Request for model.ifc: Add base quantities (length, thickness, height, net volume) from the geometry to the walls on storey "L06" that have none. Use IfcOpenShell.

First a look at what the model holds.

```python
import ifcopenshell
import ifcopenshell.util.element
import ifcopenshell.util.unit

model = ifcopenshell.open("model.ifc")
print(model.schema)
for unit_type in ("LENGTHUNIT", "AREAUNIT", "VOLUMEUNIT"):
    print(unit_type, ifcopenshell.util.unit.calculate_unit_scale(model, unit_type))
storey = next(s for s in model.by_type("IfcBuildingStorey") if s.Name == "L06")
walls = [e for e in ifcopenshell.util.element.get_decomposition(storey) if e.is_a("IfcWall")]
for e in sorted(walls, key=lambda e: e.id()):
    print(e.id(), e.is_a(), e.Name, list(ifcopenshell.util.element.get_psets(e, qtos_only=True)), sep=" | ")
```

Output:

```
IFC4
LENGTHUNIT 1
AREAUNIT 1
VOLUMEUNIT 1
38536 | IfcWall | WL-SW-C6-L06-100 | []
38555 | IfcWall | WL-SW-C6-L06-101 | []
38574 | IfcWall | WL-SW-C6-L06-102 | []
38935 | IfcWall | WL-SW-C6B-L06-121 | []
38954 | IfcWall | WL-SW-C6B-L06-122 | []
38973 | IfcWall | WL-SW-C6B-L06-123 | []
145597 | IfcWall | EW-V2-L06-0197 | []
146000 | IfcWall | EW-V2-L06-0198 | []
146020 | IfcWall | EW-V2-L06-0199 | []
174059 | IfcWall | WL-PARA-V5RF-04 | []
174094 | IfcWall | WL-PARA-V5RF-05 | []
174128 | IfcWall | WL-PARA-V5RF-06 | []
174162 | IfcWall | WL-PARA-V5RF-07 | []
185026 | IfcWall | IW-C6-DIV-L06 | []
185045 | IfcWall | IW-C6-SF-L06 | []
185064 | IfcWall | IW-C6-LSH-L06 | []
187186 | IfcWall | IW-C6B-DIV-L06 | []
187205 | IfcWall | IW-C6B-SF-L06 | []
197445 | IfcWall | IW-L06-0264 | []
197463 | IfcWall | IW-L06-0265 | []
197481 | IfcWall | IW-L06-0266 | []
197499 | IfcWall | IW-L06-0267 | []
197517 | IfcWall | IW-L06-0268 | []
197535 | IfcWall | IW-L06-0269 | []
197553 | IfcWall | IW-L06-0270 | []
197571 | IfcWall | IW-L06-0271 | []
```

```python
import ifcopenshell
import ifcopenshell.api.pset
import ifcopenshell.geom
import ifcopenshell.util.element
import ifcopenshell.util.shape
import ifcopenshell.util.unit

model = ifcopenshell.open("model.ifc")
unit_scale = ifcopenshell.util.unit.calculate_unit_scale(model)
volume_scale = ifcopenshell.util.unit.calculate_unit_scale(model, "VOLUMEUNIT")
settings = ifcopenshell.geom.settings()

storey = next(s for s in model.by_type("IfcBuildingStorey") if s.Name == "L06")
walls = [e for e in ifcopenshell.util.element.get_decomposition(storey) if e.is_a("IfcWall")]

for e in sorted(walls, key=lambda e: e.id()):
    if ifcopenshell.util.element.get_psets(e, qtos_only=True, should_inherit=False):
        continue
    # Geometry comes back in metres, in the element's own axes.
    shape = ifcopenshell.geom.create_shape(settings, e)
    values = {
        "Length": ifcopenshell.util.shape.get_x(shape.geometry) / unit_scale,
        "Width": ifcopenshell.util.shape.get_y(shape.geometry) / unit_scale,
        "Height": ifcopenshell.util.shape.get_z(shape.geometry) / unit_scale,
        "NetVolume": ifcopenshell.util.shape.get_volume(shape.geometry) / volume_scale,
    }
    qto = ifcopenshell.api.pset.add_qto(model, product=e, name="Qto_WallBaseQuantities")
    ifcopenshell.api.pset.edit_qto(model, qto=qto, properties=values)
    print(e.id(), {k: round(v, 3) for k, v in values.items()})

model.write("model_rev.ifc")
```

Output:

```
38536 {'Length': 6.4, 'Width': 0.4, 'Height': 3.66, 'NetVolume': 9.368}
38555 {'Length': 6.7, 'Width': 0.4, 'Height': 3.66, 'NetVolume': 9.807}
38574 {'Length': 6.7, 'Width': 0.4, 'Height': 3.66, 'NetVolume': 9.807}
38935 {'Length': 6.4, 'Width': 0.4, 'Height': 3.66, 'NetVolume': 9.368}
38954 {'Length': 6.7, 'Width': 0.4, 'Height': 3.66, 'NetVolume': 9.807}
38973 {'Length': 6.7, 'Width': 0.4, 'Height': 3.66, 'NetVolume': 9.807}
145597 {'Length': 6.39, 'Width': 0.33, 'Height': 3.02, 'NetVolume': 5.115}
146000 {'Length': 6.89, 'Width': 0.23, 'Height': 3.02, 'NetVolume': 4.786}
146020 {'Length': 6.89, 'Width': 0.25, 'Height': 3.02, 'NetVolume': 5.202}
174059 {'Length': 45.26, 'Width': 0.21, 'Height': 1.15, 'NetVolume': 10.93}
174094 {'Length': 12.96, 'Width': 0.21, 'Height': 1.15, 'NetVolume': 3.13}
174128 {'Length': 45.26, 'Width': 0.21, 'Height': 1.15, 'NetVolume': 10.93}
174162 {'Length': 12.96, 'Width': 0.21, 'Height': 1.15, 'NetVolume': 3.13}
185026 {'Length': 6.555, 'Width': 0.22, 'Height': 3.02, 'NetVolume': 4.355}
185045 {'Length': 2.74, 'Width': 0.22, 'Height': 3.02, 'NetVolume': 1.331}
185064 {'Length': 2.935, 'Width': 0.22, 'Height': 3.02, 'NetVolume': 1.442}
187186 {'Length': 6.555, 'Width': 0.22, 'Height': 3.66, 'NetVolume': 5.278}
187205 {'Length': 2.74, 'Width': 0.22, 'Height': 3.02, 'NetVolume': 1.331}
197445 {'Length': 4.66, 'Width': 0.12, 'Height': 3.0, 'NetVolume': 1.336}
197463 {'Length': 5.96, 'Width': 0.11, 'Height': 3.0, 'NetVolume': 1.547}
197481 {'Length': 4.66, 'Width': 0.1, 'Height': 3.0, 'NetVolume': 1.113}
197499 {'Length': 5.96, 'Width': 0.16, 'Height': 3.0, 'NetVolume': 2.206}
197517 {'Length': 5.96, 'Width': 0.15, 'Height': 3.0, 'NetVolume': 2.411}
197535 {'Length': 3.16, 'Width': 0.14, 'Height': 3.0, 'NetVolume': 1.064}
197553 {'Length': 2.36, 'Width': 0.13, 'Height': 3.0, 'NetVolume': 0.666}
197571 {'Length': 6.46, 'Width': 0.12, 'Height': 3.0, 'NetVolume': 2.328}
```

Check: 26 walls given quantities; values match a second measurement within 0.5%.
